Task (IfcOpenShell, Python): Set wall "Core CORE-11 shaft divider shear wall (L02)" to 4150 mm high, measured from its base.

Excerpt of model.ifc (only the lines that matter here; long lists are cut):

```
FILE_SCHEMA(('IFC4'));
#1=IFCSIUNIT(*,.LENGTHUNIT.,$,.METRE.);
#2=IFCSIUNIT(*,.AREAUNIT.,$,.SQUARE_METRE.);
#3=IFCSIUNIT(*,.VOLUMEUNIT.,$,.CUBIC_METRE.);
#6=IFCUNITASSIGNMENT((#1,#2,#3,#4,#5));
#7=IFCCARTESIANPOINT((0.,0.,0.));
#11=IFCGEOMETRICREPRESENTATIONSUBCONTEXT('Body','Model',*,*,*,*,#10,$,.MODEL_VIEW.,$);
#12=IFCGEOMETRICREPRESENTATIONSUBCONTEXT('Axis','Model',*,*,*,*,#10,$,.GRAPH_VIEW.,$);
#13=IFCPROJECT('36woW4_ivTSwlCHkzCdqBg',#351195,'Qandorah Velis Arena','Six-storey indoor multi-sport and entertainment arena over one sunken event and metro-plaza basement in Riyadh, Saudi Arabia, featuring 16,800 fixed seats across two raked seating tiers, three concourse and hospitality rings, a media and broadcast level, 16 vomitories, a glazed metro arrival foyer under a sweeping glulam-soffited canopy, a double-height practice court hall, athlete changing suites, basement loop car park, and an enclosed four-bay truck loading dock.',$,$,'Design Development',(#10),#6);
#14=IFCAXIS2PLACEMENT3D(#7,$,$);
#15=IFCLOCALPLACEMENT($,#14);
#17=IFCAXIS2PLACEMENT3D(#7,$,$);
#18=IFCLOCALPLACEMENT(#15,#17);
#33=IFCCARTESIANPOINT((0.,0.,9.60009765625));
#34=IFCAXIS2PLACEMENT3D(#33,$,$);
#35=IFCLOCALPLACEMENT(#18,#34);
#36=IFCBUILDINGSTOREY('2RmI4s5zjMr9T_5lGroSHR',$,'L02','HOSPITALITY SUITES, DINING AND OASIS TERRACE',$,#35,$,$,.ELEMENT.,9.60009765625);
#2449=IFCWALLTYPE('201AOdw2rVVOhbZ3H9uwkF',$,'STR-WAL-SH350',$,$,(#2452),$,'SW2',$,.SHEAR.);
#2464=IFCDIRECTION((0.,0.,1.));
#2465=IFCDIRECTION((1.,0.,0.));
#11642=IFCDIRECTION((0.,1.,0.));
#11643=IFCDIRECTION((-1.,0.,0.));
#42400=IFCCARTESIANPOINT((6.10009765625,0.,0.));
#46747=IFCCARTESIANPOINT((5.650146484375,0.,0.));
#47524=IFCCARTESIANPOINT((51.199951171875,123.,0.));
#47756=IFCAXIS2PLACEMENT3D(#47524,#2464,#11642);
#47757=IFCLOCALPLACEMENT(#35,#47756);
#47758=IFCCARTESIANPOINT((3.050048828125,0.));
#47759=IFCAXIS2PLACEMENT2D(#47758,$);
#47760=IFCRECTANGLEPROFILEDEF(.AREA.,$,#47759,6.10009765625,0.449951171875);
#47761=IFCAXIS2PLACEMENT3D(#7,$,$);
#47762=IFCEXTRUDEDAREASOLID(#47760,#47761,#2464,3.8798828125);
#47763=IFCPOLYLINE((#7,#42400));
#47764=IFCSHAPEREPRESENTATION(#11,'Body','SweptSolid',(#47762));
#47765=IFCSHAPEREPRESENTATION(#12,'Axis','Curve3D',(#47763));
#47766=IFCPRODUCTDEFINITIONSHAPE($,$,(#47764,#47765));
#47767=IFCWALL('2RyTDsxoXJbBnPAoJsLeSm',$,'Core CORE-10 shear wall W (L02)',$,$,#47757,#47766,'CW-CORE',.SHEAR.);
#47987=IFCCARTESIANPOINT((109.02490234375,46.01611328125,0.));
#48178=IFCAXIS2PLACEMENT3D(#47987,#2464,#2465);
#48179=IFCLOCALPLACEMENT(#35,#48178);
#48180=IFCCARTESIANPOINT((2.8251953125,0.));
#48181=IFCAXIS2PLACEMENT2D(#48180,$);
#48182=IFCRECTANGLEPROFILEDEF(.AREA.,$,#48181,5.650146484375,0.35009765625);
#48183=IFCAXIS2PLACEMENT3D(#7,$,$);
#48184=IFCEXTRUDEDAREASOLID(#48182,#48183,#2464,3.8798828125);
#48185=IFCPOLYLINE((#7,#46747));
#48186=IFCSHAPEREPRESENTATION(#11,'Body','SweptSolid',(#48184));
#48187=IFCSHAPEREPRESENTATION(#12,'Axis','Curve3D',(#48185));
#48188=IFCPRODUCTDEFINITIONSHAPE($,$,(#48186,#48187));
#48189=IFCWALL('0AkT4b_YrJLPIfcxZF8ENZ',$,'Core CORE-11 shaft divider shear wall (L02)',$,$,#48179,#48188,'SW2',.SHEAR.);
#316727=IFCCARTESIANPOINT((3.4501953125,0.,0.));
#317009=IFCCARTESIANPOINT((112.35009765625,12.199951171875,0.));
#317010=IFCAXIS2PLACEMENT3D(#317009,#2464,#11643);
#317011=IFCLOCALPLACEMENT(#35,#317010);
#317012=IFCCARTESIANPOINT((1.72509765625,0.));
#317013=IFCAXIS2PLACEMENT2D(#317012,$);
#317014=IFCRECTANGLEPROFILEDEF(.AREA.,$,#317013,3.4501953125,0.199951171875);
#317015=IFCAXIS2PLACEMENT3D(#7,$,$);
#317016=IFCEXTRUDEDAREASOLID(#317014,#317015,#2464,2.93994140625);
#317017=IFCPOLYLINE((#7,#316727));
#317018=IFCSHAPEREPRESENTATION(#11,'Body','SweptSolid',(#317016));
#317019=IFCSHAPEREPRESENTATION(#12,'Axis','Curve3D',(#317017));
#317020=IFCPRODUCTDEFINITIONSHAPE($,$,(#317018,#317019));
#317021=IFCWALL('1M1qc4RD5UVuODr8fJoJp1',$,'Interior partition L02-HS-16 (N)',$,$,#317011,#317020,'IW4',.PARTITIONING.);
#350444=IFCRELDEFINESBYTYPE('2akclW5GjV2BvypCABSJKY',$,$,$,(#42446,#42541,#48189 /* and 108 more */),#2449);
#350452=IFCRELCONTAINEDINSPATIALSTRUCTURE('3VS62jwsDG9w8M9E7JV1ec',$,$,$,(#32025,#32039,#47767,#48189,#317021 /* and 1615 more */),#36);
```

```python
import ifcopenshell
import ifcopenshell.geom
import ifcopenshell.util.representation
import ifcopenshell.util.shape

model = ifcopenshell.open("model.ifc")
settings = ifcopenshell.geom.settings()


def volume(element):
    """Net volume in cubic metres, openings subtracted."""
    shape = ifcopenshell.geom.create_shape(settings, element)
    return ifcopenshell.util.shape.get_volume(shape.geometry)


wall = model.by_id(48189)
before = volume(wall)

body = ifcopenshell.util.representation.get_representation(wall, "Model", "Body")
solid = body.Items[0]
old_height = solid.Depth
solid.Depth = 4.15
after = volume(wall)

print(f"height {old_height:g} -> {solid.Depth:g}, volume {before:.3f} -> {after:.3f} m3")

model.write("model_edited.ifc")
```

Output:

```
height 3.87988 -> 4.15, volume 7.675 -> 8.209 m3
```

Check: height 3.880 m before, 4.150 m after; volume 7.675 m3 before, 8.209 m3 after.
